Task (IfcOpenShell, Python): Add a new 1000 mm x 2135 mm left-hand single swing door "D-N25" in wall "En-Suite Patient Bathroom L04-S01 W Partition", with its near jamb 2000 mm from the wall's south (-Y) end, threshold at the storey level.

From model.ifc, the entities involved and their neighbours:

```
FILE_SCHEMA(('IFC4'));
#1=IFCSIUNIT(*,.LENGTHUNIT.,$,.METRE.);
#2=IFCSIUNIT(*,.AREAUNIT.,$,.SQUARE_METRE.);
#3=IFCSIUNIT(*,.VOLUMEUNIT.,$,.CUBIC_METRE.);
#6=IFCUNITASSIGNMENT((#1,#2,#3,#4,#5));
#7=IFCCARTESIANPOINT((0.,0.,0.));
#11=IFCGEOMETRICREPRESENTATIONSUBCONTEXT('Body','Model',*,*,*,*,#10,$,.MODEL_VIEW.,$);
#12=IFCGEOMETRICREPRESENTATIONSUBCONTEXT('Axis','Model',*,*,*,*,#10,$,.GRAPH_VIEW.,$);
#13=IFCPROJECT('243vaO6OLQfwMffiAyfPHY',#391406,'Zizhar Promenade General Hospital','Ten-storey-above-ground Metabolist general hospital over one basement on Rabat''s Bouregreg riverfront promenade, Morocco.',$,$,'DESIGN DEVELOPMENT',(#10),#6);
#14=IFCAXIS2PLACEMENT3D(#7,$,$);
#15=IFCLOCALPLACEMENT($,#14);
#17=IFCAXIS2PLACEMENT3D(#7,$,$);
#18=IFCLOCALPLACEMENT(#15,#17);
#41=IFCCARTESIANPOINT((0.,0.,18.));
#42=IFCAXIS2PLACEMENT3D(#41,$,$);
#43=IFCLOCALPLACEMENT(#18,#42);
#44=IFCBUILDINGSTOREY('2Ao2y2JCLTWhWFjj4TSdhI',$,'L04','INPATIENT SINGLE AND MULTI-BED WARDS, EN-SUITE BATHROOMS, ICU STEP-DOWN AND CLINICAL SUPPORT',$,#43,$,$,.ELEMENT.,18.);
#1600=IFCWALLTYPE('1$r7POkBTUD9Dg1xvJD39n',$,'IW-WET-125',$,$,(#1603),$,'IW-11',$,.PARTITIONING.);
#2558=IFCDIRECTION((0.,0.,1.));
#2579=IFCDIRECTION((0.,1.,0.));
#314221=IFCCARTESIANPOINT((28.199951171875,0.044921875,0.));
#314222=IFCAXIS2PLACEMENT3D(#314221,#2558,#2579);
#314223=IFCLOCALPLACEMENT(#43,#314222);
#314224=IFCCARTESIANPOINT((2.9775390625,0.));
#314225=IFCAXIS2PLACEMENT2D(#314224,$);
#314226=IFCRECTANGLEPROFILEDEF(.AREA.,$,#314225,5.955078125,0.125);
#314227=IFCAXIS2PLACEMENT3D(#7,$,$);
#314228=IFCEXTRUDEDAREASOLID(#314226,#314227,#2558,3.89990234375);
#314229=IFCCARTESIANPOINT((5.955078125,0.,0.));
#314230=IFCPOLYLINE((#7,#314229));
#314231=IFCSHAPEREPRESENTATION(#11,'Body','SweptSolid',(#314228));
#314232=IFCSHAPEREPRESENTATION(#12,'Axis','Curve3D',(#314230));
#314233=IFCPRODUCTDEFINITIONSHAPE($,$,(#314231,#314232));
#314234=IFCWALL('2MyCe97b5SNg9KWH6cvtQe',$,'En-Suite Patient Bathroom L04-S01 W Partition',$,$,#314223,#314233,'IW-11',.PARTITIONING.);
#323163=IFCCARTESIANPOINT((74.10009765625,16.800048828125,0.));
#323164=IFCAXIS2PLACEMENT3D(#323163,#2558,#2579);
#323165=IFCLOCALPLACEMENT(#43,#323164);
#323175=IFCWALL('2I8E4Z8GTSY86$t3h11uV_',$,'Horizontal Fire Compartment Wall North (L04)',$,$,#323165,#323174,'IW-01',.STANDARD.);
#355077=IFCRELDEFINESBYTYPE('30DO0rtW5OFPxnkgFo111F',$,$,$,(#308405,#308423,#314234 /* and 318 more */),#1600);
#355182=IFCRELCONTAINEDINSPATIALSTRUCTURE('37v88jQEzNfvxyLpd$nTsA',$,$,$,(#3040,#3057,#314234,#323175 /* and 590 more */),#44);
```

```python
import numpy as np
import ifcopenshell
import ifcopenshell.api.feature
import ifcopenshell.api.geometry
import ifcopenshell.api.root
import ifcopenshell.api.spatial
import ifcopenshell.geom
import ifcopenshell.util.element
import ifcopenshell.util.placement
import ifcopenshell.util.representation
import ifcopenshell.util.shape
import ifcopenshell.util.unit

model = ifcopenshell.open("model.ifc")
unit_scale = ifcopenshell.util.unit.calculate_unit_scale(model)
settings = ifcopenshell.geom.settings()


def volume(element):
    """Net volume in cubic metres, openings subtracted."""
    shape = ifcopenshell.geom.create_shape(settings, element)
    return ifcopenshell.util.shape.get_volume(shape.geometry)


wall = model.by_guid("2MyCe97b5SNg9KWH6cvtQe")
storey = ifcopenshell.util.element.get_container(wall, ifc_class="IfcBuildingStorey")
context = ifcopenshell.util.representation.get_context(model, "Model", "Body", "MODEL_VIEW")
before = volume(wall)

width, height, from_end, sill = 1, 2.135, 2, 0.0  # metres

# The wall runs along its own X axis, and the end named is its -X end.
wall_shape = ifcopenshell.geom.create_shape(settings, wall)
x, y, z = ifcopenshell.util.shape.get_vertices(wall_shape.geometry).T
start = x.min() + from_end
face, thickness = float(y.min()), float(y.max() - y.min())
wall_matrix = ifcopenshell.util.placement.get_local_placement(wall.ObjectPlacement)
level = ifcopenshell.util.placement.get_local_placement(storey.ObjectPlacement)[2, 3]


def in_wall(x, y):
    """Placement at x, y metres in the wall's axes, at sill height."""
    matrix = wall_matrix.copy()
    matrix[:, 3] = wall_matrix @ np.array([x / unit_scale, y / unit_scale, 0.0, 1.0])
    matrix[2, 3] = level + sill / unit_scale
    return matrix


# Opening: a box that overshoots both wall faces by 50 mm.
opening = ifcopenshell.api.root.create_entity(model, ifc_class="IfcOpeningElement", predefined_type="OPENING")
box = ifcopenshell.api.geometry.add_wall_representation(
    model, context=context, length=width, height=height, thickness=thickness + 0.1
)
ifcopenshell.api.geometry.assign_representation(model, product=opening, representation=box)
ifcopenshell.api.geometry.edit_object_placement(model, product=opening, matrix=in_wall(start, face - 0.05), is_si=False)
ifcopenshell.api.feature.add_feature(model, feature=opening, element=wall)

door = ifcopenshell.api.root.create_entity(model, ifc_class="IfcDoor", name="D-N25", predefined_type="DOOR")
door.OverallWidth, door.OverallHeight = width / unit_scale, height / unit_scale
door.OperationType = "SINGLE_SWING_LEFT"
body = ifcopenshell.api.geometry.add_door_representation(
    model,
    context=context,
    overall_width=door.OverallWidth,
    overall_height=door.OverallHeight,
    operation_type="SINGLE_SWING_LEFT",
    lining_properties={"LiningDepth": thickness / unit_scale, "ThresholdDepth": thickness / unit_scale},
)
ifcopenshell.api.geometry.assign_representation(model, product=door, representation=body)
ifcopenshell.api.spatial.assign_container(model, products=[door], relating_structure=storey)
ifcopenshell.api.feature.add_filling(model, opening=opening, element=door)

# The lining spans the wall, so the door starts at the wall face.
ifcopenshell.api.geometry.edit_object_placement(model, product=door, matrix=in_wall(start, face), is_si=False)

after = volume(wall)

print(f"wall volume {before:.3f} -> {after:.3f} m3")

model.write("model_edited.ifc")
```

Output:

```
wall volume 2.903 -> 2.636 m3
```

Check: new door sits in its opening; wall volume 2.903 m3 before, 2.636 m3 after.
